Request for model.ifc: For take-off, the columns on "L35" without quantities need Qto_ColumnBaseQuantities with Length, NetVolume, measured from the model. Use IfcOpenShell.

First a look at what the model holds.

```python
import ifcopenshell
import ifcopenshell.util.element
import ifcopenshell.util.unit

model = ifcopenshell.open("model.ifc")
print(model.schema)
for unit_type in ("LENGTHUNIT", "AREAUNIT", "VOLUMEUNIT"):
    print(unit_type, ifcopenshell.util.unit.calculate_unit_scale(model, unit_type))
storey = next(s for s in model.by_type("IfcBuildingStorey") if s.Name == "L35")
columns = [e for e in ifcopenshell.util.element.get_decomposition(storey) if e.is_a("IfcColumn")]
for e in sorted(columns, key=lambda e: e.id()):
    print(e.id(), e.is_a(), e.Name, list(ifcopenshell.util.element.get_psets(e, qtos_only=True)), sep=" | ")
```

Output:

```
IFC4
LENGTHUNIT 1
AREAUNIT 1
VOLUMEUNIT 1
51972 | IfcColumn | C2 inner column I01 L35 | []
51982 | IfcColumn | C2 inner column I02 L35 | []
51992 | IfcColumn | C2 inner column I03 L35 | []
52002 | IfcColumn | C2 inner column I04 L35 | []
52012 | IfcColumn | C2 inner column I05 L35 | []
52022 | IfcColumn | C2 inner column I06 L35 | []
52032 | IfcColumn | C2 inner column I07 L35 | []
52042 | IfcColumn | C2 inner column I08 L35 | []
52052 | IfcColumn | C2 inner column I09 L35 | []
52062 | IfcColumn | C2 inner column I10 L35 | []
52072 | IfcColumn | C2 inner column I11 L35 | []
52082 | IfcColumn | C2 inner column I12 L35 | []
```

```python
import ifcopenshell
import ifcopenshell.api.pset
import ifcopenshell.geom
import ifcopenshell.util.element
import ifcopenshell.util.shape
import ifcopenshell.util.unit

model = ifcopenshell.open("model.ifc")
unit_scale = ifcopenshell.util.unit.calculate_unit_scale(model)
volume_scale = ifcopenshell.util.unit.calculate_unit_scale(model, "VOLUMEUNIT")
settings = ifcopenshell.geom.settings()

storey = next(s for s in model.by_type("IfcBuildingStorey") if s.Name == "L35")
columns = [e for e in ifcopenshell.util.element.get_decomposition(storey) if e.is_a("IfcColumn")]

for e in sorted(columns, key=lambda e: e.id()):
    if ifcopenshell.util.element.get_psets(e, qtos_only=True, should_inherit=False):
        continue
    # Geometry comes back in metres, in the element's own axes.
    shape = ifcopenshell.geom.create_shape(settings, e)
    values = {
        "Length": ifcopenshell.util.shape.get_z(shape.geometry) / unit_scale,
        "NetVolume": ifcopenshell.util.shape.get_volume(shape.geometry) / volume_scale,
    }
    qto = ifcopenshell.api.pset.add_qto(model, product=e, name="Qto_ColumnBaseQuantities")
    ifcopenshell.api.pset.edit_qto(model, qto=qto, properties=values)
    print(e.id(), {k: round(v, 3) for k, v in values.items()})

model.write("model_rev.ifc")
```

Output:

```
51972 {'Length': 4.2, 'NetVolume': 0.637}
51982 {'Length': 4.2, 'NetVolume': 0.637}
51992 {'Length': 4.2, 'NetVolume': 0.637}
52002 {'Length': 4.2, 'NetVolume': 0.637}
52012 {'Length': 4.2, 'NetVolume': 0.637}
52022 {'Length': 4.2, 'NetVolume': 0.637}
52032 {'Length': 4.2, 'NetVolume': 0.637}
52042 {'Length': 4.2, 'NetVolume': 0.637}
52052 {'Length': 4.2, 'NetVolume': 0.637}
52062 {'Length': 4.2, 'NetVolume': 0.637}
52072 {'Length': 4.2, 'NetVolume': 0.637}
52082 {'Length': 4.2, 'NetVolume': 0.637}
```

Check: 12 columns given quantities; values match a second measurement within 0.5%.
